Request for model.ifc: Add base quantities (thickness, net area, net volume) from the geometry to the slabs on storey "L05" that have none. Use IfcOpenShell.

First a look at what the model holds.

```python
import ifcopenshell
import ifcopenshell.util.element
import ifcopenshell.util.unit

model = ifcopenshell.open("model.ifc")
print(model.schema)
for unit_type in ("LENGTHUNIT", "AREAUNIT", "VOLUMEUNIT"):
    print(unit_type, ifcopenshell.util.unit.calculate_unit_scale(model, unit_type))
storey = next(s for s in model.by_type("IfcBuildingStorey") if s.Name == "L05")
slabs = [e for e in ifcopenshell.util.element.get_decomposition(storey) if e.is_a("IfcSlab")]
for e in sorted(slabs, key=lambda e: e.id()):
    print(e.id(), e.is_a(), e.Name, list(ifcopenshell.util.element.get_psets(e, qtos_only=True)), sep=" | ")
```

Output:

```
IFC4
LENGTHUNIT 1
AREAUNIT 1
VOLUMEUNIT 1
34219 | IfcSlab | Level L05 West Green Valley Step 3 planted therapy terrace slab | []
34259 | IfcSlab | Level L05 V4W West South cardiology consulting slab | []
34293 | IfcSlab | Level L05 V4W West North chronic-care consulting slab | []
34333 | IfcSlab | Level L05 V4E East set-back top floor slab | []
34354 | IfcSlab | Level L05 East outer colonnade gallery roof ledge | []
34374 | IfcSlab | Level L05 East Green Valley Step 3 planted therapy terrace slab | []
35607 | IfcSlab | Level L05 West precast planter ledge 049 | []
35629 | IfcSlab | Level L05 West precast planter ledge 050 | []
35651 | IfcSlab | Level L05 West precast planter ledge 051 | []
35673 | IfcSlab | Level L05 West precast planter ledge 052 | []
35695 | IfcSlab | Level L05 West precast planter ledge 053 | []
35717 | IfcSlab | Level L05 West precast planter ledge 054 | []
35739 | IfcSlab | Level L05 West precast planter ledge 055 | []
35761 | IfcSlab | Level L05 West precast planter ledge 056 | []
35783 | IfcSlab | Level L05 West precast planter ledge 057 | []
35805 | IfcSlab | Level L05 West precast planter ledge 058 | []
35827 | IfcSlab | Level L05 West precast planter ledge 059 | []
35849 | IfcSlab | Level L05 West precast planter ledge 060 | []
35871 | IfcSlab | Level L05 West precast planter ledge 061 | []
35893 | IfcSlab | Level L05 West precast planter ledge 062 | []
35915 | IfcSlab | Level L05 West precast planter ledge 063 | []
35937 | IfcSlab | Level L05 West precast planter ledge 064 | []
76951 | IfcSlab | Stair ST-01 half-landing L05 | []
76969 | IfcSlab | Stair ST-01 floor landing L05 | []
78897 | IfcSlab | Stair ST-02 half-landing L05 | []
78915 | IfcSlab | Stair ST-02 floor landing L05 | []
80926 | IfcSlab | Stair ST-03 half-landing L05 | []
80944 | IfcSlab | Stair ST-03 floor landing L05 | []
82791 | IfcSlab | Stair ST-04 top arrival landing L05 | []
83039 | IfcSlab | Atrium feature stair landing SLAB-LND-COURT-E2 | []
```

```python
import ifcopenshell
import ifcopenshell.api.pset
import ifcopenshell.geom
import ifcopenshell.util.element
import ifcopenshell.util.shape
import ifcopenshell.util.unit

model = ifcopenshell.open("model.ifc")
unit_scale = ifcopenshell.util.unit.calculate_unit_scale(model)
area_scale = ifcopenshell.util.unit.calculate_unit_scale(model, "AREAUNIT")
volume_scale = ifcopenshell.util.unit.calculate_unit_scale(model, "VOLUMEUNIT")
settings = ifcopenshell.geom.settings()

storey = next(s for s in model.by_type("IfcBuildingStorey") if s.Name == "L05")
slabs = [e for e in ifcopenshell.util.element.get_decomposition(storey) if e.is_a("IfcSlab")]

for e in sorted(slabs, key=lambda e: e.id()):
    if ifcopenshell.util.element.get_psets(e, qtos_only=True, should_inherit=False):
        continue
    # Geometry comes back in metres, in the element's own axes.
    shape = ifcopenshell.geom.create_shape(settings, e)
    values = {
        "Width": ifcopenshell.util.shape.get_z(shape.geometry) / unit_scale,
        "NetArea": ifcopenshell.util.shape.get_footprint_area(shape.geometry) / area_scale,
        "NetVolume": ifcopenshell.util.shape.get_volume(shape.geometry) / volume_scale,
    }
    qto = ifcopenshell.api.pset.add_qto(model, product=e, name="Qto_SlabBaseQuantities")
    ifcopenshell.api.pset.edit_qto(model, qto=qto, properties=values)
    print(e.id(), {k: round(v, 3) for k, v in values.items()})

model.write("model_edited.ifc")
```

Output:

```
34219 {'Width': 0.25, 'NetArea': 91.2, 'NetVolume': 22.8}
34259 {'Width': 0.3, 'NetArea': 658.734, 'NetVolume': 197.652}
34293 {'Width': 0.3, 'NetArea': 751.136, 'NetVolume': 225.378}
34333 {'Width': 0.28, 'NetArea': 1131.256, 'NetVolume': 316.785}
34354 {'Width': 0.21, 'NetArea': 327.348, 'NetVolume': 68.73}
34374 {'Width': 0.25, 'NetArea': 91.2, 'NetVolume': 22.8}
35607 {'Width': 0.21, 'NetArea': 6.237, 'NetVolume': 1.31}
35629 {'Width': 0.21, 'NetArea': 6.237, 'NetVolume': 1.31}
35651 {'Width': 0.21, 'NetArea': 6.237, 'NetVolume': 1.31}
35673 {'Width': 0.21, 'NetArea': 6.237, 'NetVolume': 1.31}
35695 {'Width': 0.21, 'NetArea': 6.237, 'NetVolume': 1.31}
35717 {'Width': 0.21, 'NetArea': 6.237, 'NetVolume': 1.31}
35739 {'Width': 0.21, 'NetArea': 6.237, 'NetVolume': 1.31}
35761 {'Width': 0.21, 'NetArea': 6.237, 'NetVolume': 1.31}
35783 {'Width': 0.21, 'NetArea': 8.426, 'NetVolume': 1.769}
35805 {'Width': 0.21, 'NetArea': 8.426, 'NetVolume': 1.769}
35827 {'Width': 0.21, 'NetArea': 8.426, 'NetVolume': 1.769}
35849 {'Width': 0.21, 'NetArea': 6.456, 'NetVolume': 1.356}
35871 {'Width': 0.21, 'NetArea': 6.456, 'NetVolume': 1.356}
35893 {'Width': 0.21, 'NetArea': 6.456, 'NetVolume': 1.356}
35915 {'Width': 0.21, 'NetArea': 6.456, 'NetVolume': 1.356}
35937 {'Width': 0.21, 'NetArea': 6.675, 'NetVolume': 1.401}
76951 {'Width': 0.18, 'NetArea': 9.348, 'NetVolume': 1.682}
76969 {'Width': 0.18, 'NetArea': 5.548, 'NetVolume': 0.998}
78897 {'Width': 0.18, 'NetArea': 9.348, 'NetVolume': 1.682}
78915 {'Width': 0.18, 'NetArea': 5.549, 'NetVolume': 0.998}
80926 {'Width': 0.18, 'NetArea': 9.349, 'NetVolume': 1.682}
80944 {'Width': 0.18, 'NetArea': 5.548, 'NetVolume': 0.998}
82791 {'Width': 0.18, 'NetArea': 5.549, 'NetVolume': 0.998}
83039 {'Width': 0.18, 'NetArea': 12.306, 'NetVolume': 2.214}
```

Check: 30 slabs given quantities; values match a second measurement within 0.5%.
